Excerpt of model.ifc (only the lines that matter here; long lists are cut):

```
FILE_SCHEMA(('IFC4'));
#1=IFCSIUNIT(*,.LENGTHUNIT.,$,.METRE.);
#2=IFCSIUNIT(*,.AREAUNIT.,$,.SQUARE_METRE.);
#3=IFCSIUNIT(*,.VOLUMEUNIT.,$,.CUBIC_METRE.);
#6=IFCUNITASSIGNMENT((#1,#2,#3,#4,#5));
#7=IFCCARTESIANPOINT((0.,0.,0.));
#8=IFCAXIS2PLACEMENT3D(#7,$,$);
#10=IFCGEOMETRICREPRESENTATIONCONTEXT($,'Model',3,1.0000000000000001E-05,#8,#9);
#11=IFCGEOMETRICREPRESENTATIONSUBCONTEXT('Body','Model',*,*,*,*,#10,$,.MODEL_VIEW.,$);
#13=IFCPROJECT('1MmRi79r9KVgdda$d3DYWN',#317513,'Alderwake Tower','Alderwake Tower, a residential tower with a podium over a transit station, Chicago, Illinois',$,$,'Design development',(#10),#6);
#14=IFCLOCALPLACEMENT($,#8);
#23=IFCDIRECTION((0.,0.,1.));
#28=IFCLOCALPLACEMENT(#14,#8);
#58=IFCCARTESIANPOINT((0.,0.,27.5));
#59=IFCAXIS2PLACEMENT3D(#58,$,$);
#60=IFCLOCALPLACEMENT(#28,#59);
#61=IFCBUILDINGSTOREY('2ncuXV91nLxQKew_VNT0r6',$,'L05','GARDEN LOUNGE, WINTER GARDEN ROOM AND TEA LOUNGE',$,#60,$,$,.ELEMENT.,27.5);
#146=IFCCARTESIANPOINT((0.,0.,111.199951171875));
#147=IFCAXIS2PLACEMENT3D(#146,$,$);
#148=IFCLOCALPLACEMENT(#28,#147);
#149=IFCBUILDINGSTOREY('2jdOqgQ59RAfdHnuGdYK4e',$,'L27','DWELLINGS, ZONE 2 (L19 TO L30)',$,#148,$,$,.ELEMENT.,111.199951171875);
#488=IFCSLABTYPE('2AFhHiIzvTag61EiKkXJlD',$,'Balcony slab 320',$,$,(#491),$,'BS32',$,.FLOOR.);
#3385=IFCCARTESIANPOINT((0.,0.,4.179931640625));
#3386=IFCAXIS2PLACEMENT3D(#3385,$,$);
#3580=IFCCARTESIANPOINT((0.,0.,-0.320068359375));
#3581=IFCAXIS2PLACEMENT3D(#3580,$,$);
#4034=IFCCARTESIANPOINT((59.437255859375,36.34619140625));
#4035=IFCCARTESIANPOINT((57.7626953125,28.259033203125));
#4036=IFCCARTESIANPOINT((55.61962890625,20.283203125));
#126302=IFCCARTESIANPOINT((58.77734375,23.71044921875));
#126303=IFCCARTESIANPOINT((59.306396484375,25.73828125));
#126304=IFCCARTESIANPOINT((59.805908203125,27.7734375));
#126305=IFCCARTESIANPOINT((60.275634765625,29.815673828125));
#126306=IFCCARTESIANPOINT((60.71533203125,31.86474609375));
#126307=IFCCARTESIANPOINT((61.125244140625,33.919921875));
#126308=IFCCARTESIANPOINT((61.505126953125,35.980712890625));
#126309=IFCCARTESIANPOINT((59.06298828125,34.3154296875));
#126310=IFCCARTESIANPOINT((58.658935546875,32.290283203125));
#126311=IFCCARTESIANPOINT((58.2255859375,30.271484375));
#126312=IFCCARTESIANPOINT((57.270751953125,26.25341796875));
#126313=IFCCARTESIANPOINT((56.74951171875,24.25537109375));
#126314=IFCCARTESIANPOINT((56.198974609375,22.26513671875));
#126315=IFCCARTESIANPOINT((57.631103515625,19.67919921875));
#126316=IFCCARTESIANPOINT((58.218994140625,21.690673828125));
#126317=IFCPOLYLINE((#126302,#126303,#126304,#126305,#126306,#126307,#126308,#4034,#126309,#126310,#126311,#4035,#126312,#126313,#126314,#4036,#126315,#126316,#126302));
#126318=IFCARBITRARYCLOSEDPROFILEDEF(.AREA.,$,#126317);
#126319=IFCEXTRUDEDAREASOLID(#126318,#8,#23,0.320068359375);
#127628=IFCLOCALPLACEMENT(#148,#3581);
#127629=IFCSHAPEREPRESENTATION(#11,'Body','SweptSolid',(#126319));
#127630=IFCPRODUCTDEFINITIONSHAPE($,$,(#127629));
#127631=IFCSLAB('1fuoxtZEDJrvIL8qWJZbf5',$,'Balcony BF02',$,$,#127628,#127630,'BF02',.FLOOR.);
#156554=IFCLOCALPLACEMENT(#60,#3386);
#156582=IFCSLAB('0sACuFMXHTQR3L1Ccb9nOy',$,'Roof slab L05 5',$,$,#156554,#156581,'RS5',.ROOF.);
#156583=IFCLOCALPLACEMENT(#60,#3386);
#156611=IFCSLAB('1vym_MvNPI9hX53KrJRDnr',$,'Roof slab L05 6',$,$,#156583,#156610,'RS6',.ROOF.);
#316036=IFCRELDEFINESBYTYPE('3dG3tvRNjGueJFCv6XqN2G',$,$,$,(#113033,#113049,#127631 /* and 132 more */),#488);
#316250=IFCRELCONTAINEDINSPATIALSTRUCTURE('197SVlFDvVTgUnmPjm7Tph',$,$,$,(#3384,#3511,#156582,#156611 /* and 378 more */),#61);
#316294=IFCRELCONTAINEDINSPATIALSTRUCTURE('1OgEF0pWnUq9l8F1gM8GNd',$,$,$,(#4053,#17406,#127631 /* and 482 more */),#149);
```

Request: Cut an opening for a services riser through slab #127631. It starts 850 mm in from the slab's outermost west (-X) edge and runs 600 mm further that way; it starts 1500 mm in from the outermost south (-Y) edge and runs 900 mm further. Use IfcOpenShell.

```python
import numpy as np
import ifcopenshell
import ifcopenshell.api.feature
import ifcopenshell.api.geometry
import ifcopenshell.api.root
import ifcopenshell.geom
import ifcopenshell.util.placement
import ifcopenshell.util.representation
import ifcopenshell.util.shape
import ifcopenshell.util.unit

model = ifcopenshell.open("model.ifc")
unit_scale = ifcopenshell.util.unit.calculate_unit_scale(model)
settings = ifcopenshell.geom.settings()


def volume(element):
    """Net volume in cubic metres, openings subtracted."""
    shape = ifcopenshell.geom.create_shape(settings, element)
    return ifcopenshell.util.shape.get_volume(shape.geometry)


slab = model.by_id(127631)
before = volume(slab)

# Extent in the slab's own axes, in metres. The edges named are its -X and -Y sides.
slab_shape = ifcopenshell.geom.create_shape(settings, slab)
vertices = ifcopenshell.util.shape.get_vertices(slab_shape.geometry)
x_min, y_min, bottom = vertices.min(axis=0)
top = vertices[:, 2].max()

opening = ifcopenshell.api.root.create_entity(model, ifc_class="IfcOpeningElement", name="Services riser opening", predefined_type="OPENING")
context = ifcopenshell.util.representation.get_context(model, "Model", "Body", "MODEL_VIEW")
width, depth = 0.6, 0.9
outline = [(0.0, 0.0), (width, 0.0), (width, depth), (0.0, depth), (0.0, 0.0)]
# Overshoot both faces by 50 mm so the cut is clean.
shape = ifcopenshell.api.geometry.add_slab_representation(
    model, context=context, depth=top - bottom + 0.1, polyline=outline
)
ifcopenshell.api.geometry.assign_representation(model, product=opening, representation=shape)

matrix = ifcopenshell.util.placement.get_local_placement(slab.ObjectPlacement)
matrix[:, 3] = matrix @ np.append(np.array([x_min + 0.85, y_min + 1.5, bottom - 0.05]) / unit_scale, 1.0)
ifcopenshell.api.geometry.edit_object_placement(model, product=opening, matrix=matrix, is_si=False)
ifcopenshell.api.feature.add_feature(model, feature=opening, element=slab)

after = volume(slab)

print(f"slab volume {before:.3f} -> {after:.3f} m3")

model.write("model-out.ifc")
```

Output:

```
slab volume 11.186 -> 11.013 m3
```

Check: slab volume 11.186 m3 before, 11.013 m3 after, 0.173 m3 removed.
